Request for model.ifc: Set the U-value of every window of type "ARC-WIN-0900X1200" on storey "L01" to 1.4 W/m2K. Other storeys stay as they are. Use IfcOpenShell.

First a look at what the model holds.

```python
import ifcopenshell
import ifcopenshell.util.element

model = ifcopenshell.open("model.ifc")
print(model.schema)
storey = next(s for s in model.by_type("IfcBuildingStorey") if s.Name == "L01")
windows = [e for e in ifcopenshell.util.element.get_decomposition(storey) if e.is_a("IfcWindow")]
seen = {}
for e in windows:
    element_type = ifcopenshell.util.element.get_type(e)
    key = (element_type.Name if element_type != e and element_type else None, ifcopenshell.util.element.get_pset(e, "Pset_WindowCommon", "ThermalTransmittance"))
    seen[key] = seen.get(key, 0) + 1
for (name, value), count in sorted(seen.items(), key=str):
    print(count, "x", name, "|", value)
```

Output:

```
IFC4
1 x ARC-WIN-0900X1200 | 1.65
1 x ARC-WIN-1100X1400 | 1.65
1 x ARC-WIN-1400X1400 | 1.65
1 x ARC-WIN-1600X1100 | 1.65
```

```python
import ifcopenshell
import ifcopenshell.api.pset
import ifcopenshell.util.element

model = ifcopenshell.open("model.ifc")

storey = next(s for s in model.by_type("IfcBuildingStorey") if s.Name == "L01")
windows = [e for e in ifcopenshell.util.element.get_decomposition(storey) if e.is_a("IfcWindow")]

count = 0
for e in windows:
    element_type = ifcopenshell.util.element.get_type(e)
    if element_type in (None, e) or element_type.Name != "ARC-WIN-0900X1200":
        continue
    # add_pset returns the element's existing set when there is one.
    pset = ifcopenshell.api.pset.add_pset(model, product=e, name="Pset_WindowCommon")
    ifcopenshell.api.pset.edit_pset(model, pset=pset, properties={"ThermalTransmittance": 1.4})
    count += 1

print(count, "windows updated")

model.write("model_updated.ifc")
```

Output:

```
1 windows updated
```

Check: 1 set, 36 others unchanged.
